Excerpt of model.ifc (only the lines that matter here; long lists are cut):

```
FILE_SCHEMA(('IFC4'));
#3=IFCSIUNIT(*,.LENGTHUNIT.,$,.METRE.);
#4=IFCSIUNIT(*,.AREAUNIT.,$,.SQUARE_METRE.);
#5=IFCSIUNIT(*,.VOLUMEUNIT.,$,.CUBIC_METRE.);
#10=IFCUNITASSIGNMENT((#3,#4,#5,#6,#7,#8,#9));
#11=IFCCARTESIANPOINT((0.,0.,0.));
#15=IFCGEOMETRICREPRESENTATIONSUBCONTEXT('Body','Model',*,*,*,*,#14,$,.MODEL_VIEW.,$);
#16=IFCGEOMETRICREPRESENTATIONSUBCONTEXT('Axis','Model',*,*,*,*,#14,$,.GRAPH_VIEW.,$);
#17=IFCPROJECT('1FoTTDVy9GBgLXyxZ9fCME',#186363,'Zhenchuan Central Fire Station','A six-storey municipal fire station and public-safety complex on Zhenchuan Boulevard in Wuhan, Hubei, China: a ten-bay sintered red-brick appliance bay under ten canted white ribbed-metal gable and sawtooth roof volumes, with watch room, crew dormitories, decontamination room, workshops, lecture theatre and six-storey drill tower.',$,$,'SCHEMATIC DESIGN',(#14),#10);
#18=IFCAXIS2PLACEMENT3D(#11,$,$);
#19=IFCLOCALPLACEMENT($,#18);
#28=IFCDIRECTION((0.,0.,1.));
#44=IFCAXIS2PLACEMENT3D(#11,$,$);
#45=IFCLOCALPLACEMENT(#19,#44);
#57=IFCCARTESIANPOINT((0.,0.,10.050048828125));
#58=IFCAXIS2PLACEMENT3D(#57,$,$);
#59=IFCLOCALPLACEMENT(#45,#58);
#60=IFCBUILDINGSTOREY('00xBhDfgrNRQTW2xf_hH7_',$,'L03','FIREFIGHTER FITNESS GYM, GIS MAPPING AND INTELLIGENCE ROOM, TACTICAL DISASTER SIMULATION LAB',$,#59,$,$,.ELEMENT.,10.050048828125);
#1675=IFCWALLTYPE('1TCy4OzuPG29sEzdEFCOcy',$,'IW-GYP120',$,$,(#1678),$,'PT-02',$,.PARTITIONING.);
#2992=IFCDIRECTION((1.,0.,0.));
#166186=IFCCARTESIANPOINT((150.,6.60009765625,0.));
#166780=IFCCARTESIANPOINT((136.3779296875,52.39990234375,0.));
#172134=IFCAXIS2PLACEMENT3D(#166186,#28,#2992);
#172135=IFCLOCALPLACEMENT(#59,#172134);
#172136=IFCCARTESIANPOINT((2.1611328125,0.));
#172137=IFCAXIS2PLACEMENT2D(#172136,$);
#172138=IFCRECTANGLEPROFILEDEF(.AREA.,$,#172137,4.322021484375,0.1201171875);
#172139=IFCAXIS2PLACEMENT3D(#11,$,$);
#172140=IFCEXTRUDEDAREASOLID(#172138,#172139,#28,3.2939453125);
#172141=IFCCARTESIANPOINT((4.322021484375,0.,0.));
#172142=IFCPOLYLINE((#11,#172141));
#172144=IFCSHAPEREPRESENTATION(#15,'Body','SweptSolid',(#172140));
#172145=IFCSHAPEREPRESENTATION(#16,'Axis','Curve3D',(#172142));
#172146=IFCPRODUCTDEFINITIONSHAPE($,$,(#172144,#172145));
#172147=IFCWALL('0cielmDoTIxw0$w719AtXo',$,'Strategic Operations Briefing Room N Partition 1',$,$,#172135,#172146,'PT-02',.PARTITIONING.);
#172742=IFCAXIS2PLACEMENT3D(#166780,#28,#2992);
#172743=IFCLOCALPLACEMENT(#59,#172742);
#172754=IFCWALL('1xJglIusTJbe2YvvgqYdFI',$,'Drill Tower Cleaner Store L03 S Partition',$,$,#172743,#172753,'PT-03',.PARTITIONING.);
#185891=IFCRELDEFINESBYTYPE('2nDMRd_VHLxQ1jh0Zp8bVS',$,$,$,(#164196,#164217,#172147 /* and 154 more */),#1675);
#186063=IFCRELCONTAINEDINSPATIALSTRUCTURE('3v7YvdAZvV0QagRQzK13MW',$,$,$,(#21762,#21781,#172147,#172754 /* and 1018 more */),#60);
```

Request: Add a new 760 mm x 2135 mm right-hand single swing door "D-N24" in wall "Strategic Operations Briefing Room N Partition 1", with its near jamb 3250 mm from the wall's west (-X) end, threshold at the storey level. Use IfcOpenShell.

```python
import numpy as np
import ifcopenshell
import ifcopenshell.api.feature
import ifcopenshell.api.geometry
import ifcopenshell.api.root
import ifcopenshell.api.spatial
import ifcopenshell.geom
import ifcopenshell.util.element
import ifcopenshell.util.placement
import ifcopenshell.util.representation
import ifcopenshell.util.shape
import ifcopenshell.util.unit

model = ifcopenshell.open("model.ifc")
unit_scale = ifcopenshell.util.unit.calculate_unit_scale(model)
settings = ifcopenshell.geom.settings()


def volume(element):
    """Net volume in cubic metres, openings subtracted."""
    shape = ifcopenshell.geom.create_shape(settings, element)
    return ifcopenshell.util.shape.get_volume(shape.geometry)


wall = model.by_guid("0cielmDoTIxw0$w719AtXo")
storey = ifcopenshell.util.element.get_container(wall, ifc_class="IfcBuildingStorey")
context = ifcopenshell.util.representation.get_context(model, "Model", "Body", "MODEL_VIEW")
before = volume(wall)

width, height, from_end, sill = 0.76, 2.135, 3.25, 0.0  # metres

# The wall runs along its own X axis, and the end named is its -X end.
wall_shape = ifcopenshell.geom.create_shape(settings, wall)
x, y, z = ifcopenshell.util.shape.get_vertices(wall_shape.geometry).T
start = x.min() + from_end
face, thickness = float(y.min()), float(y.max() - y.min())
wall_matrix = ifcopenshell.util.placement.get_local_placement(wall.ObjectPlacement)
level = ifcopenshell.util.placement.get_local_placement(storey.ObjectPlacement)[2, 3]


def in_wall(x, y):
    """Placement at x, y metres in the wall's axes, at sill height."""
    matrix = wall_matrix.copy()
    matrix[:, 3] = wall_matrix @ np.array([x / unit_scale, y / unit_scale, 0.0, 1.0])
    matrix[2, 3] = level + sill / unit_scale
    return matrix


# Opening: a box that overshoots both wall faces by 50 mm.
opening = ifcopenshell.api.root.create_entity(model, ifc_class="IfcOpeningElement", predefined_type="OPENING")
box = ifcopenshell.api.geometry.add_wall_representation(
    model, context=context, length=width, height=height, thickness=thickness + 0.1
)
ifcopenshell.api.geometry.assign_representation(model, product=opening, representation=box)
ifcopenshell.api.geometry.edit_object_placement(model, product=opening, matrix=in_wall(start, face - 0.05), is_si=False)
ifcopenshell.api.feature.add_feature(model, feature=opening, element=wall)

door = ifcopenshell.api.root.create_entity(model, ifc_class="IfcDoor", name="D-N24", predefined_type="DOOR")
door.OverallWidth, door.OverallHeight = width / unit_scale, height / unit_scale
door.OperationType = "SINGLE_SWING_RIGHT"
body = ifcopenshell.api.geometry.add_door_representation(
    model,
    context=context,
    overall_width=door.OverallWidth,
    overall_height=door.OverallHeight,
    operation_type="SINGLE_SWING_RIGHT",
    lining_properties={"LiningDepth": thickness / unit_scale, "ThresholdDepth": thickness / unit_scale},
)
ifcopenshell.api.geometry.assign_representation(model, product=door, representation=body)
ifcopenshell.api.spatial.assign_container(model, products=[door], relating_structure=storey)
ifcopenshell.api.feature.add_filling(model, opening=opening, element=door)

# The lining spans the wall, so the door starts at the wall face.
ifcopenshell.api.geometry.edit_object_placement(model, product=door, matrix=in_wall(start, face), is_si=False)

after = volume(wall)

print(f"wall volume {before:.3f} -> {after:.3f} m3")

model.write("model-out.ifc")
```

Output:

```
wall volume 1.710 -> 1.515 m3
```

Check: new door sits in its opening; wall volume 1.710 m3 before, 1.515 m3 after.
